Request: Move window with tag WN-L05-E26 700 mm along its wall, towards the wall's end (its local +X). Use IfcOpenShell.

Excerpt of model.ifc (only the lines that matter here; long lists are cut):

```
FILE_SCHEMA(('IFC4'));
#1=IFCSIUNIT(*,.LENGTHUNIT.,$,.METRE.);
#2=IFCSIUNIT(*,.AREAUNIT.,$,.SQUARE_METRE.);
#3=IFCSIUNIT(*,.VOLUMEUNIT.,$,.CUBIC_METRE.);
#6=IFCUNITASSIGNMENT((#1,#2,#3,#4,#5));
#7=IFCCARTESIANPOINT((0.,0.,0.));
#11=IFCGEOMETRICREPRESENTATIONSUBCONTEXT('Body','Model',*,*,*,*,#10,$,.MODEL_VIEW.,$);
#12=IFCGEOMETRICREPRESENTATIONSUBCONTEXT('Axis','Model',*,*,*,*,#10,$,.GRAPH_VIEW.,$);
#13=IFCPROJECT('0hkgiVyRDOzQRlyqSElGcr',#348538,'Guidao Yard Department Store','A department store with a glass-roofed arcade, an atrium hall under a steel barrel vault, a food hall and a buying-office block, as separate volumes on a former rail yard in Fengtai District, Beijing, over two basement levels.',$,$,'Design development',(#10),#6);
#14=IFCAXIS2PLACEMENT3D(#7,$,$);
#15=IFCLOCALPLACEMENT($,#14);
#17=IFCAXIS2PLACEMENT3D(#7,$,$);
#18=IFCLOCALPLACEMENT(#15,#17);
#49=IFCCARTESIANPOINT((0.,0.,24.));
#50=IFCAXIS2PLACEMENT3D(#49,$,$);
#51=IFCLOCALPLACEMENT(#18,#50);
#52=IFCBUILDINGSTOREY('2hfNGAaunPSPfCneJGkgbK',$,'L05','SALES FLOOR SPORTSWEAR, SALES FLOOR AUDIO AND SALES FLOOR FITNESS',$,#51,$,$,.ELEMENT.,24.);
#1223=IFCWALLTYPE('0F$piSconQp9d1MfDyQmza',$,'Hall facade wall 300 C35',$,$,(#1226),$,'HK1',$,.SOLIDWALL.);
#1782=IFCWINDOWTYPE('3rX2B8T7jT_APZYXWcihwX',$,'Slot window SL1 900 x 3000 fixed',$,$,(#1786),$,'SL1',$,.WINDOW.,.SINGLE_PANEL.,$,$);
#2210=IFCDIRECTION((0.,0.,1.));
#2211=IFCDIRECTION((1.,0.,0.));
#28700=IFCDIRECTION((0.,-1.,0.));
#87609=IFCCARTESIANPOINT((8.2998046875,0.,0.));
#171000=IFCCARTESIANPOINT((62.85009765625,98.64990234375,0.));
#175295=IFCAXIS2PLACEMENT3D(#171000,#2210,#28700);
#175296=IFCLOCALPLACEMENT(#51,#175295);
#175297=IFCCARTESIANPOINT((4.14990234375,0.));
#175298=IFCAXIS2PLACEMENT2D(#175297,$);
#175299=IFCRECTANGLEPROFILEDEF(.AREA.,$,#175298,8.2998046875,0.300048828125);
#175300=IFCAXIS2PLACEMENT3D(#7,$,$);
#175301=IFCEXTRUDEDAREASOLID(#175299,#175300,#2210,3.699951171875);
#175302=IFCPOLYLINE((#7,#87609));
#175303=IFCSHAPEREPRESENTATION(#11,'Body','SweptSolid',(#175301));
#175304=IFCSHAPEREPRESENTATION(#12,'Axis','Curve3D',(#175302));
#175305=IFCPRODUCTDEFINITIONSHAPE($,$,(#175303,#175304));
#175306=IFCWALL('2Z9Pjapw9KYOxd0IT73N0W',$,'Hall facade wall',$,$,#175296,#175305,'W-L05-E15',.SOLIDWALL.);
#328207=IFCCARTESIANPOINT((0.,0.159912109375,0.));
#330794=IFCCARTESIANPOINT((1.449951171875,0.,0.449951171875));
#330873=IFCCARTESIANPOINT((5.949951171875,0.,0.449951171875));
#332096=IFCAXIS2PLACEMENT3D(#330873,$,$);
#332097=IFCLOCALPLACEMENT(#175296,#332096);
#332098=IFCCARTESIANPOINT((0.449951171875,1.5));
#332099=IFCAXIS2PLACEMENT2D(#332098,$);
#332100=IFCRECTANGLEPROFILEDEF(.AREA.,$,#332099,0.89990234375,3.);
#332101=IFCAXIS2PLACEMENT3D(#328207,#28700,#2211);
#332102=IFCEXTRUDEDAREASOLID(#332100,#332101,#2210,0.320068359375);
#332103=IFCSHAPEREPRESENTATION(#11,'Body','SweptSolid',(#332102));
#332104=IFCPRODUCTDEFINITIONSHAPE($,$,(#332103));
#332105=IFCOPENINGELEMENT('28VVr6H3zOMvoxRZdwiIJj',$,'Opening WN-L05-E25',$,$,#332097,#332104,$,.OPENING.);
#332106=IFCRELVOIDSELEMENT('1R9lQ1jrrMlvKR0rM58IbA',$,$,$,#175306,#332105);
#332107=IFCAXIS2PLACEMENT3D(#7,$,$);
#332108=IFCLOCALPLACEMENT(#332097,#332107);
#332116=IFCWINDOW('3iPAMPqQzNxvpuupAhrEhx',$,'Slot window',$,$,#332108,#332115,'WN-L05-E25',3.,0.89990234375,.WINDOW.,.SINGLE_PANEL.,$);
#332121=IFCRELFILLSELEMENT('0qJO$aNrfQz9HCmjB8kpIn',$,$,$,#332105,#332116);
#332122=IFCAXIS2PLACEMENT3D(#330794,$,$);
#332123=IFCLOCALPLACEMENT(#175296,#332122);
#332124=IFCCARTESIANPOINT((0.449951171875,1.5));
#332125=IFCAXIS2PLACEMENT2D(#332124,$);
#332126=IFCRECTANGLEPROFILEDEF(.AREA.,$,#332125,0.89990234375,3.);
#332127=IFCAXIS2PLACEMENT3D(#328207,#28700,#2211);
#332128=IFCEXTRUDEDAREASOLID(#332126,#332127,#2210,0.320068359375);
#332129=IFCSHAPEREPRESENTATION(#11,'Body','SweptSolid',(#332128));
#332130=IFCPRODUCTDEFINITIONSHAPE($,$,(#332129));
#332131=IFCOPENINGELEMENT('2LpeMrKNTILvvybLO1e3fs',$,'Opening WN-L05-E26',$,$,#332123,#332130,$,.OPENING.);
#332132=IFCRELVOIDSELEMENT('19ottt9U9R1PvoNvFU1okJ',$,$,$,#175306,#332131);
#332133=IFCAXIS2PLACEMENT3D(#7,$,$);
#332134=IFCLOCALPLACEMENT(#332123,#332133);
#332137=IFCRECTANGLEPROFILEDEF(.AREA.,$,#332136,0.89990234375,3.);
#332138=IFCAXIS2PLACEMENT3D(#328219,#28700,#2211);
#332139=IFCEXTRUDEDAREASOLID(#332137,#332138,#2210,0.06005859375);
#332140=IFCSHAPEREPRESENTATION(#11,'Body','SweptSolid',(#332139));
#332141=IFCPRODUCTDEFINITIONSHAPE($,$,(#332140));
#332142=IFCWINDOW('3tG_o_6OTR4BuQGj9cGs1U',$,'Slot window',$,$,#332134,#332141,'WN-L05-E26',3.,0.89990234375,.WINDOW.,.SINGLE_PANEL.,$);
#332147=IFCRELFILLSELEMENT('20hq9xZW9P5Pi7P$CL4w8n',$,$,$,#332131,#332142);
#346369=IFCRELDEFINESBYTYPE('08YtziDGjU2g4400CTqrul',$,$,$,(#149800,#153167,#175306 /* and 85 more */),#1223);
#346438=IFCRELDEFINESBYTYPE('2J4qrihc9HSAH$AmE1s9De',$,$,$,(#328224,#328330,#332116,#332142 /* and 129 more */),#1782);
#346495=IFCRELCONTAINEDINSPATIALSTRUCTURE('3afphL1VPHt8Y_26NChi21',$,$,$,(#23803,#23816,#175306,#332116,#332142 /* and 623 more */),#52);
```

```python
import ifcopenshell
import ifcopenshell.api.geometry
import ifcopenshell.util.placement
import ifcopenshell.util.unit

model = ifcopenshell.open("model.ifc")
unit_scale = ifcopenshell.util.unit.calculate_unit_scale(model)

window = model.by_guid("3tG_o_6OTR4BuQGj9cGs1U")
opening = window.FillsVoids[0].RelatingOpeningElement
wall = opening.VoidsElements[0].RelatingBuildingElement

wall_matrix = ifcopenshell.util.placement.get_local_placement(wall.ObjectPlacement)
shift = wall_matrix[:3, 0] * 0.7 / unit_scale
before = ifcopenshell.util.placement.get_local_placement(window.ObjectPlacement)[:3, 3].copy()

# The window is placed relative to its opening, so it follows when the opening moves.
matrix = ifcopenshell.util.placement.get_local_placement(opening.ObjectPlacement)
matrix[:3, 3] += shift
ifcopenshell.api.geometry.edit_object_placement(
    model, product=opening, matrix=matrix, is_si=False, should_transform_children=True
)

after = ifcopenshell.util.placement.get_local_placement(window.ObjectPlacement)[:3, 3]
print("window moved by", (after - before).round(3) + 0.0)

model.write("model_edited.ifc")
```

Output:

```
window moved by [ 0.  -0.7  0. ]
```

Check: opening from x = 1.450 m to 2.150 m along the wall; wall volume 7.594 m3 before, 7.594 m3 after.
